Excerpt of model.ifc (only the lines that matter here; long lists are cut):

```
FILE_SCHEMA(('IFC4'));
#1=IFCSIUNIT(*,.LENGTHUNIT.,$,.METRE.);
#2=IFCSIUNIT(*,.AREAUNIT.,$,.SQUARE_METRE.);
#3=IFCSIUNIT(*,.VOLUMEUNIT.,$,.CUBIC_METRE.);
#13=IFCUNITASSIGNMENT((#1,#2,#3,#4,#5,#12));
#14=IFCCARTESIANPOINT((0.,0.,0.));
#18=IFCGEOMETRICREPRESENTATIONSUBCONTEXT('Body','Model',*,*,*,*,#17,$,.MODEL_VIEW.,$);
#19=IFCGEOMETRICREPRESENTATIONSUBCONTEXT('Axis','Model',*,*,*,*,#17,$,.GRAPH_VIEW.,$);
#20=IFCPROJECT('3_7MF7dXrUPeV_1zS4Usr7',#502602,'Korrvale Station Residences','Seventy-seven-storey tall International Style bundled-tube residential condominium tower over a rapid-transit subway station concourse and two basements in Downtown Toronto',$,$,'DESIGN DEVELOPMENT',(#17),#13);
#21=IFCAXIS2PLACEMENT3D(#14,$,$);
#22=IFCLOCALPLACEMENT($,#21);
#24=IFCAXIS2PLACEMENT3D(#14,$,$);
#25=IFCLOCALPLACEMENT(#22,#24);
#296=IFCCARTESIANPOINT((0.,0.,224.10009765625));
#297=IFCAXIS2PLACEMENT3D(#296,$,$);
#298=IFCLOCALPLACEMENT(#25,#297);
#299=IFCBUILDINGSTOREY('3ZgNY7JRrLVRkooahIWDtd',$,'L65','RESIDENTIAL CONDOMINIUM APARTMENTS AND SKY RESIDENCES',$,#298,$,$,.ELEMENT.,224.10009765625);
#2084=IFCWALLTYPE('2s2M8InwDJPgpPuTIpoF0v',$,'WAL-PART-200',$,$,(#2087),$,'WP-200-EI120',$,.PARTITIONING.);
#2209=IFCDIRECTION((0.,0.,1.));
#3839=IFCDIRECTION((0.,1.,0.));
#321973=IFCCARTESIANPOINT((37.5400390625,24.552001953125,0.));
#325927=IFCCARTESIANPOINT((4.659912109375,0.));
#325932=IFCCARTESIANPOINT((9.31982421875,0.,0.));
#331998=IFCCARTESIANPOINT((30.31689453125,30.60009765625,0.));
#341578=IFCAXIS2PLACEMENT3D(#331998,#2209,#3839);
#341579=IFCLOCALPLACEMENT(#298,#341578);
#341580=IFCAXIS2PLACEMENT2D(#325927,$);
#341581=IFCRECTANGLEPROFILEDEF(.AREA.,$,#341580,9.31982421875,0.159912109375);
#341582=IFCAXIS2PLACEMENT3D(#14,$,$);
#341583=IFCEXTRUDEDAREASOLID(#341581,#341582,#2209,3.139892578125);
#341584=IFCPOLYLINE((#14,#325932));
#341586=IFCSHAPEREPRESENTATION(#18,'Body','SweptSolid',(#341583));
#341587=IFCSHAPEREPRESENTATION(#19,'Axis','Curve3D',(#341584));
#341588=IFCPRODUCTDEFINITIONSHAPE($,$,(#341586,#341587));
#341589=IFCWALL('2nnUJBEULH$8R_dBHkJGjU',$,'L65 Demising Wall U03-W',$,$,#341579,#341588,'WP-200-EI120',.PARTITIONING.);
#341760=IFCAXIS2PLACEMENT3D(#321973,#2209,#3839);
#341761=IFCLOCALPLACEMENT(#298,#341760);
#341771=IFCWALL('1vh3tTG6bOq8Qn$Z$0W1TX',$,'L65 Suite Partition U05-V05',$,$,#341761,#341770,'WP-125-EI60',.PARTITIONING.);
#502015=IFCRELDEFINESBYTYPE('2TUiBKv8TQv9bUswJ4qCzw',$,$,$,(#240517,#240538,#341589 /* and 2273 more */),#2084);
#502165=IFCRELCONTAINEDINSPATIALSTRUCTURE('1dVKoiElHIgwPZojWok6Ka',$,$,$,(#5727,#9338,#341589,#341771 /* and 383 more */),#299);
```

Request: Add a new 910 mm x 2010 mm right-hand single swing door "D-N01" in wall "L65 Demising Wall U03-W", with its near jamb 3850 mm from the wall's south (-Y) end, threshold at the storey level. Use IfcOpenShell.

```python
import numpy as np
import ifcopenshell
import ifcopenshell.api.feature
import ifcopenshell.api.geometry
import ifcopenshell.api.root
import ifcopenshell.api.spatial
import ifcopenshell.geom
import ifcopenshell.util.element
import ifcopenshell.util.placement
import ifcopenshell.util.representation
import ifcopenshell.util.shape
import ifcopenshell.util.unit

model = ifcopenshell.open("model.ifc")
unit_scale = ifcopenshell.util.unit.calculate_unit_scale(model)
settings = ifcopenshell.geom.settings()


def volume(element):
    """Net volume in cubic metres, openings subtracted."""
    shape = ifcopenshell.geom.create_shape(settings, element)
    return ifcopenshell.util.shape.get_volume(shape.geometry)


wall = model.by_guid("2nnUJBEULH$8R_dBHkJGjU")
storey = ifcopenshell.util.element.get_container(wall, ifc_class="IfcBuildingStorey")
context = ifcopenshell.util.representation.get_context(model, "Model", "Body", "MODEL_VIEW")
before = volume(wall)

width, height, from_end, sill = 0.91, 2.01, 3.85, 0.0  # metres

# The wall runs along its own X axis, and the end named is its -X end.
wall_shape = ifcopenshell.geom.create_shape(settings, wall)
x, y, z = ifcopenshell.util.shape.get_vertices(wall_shape.geometry).T
start = x.min() + from_end
face, thickness = float(y.min()), float(y.max() - y.min())
wall_matrix = ifcopenshell.util.placement.get_local_placement(wall.ObjectPlacement)
level = ifcopenshell.util.placement.get_local_placement(storey.ObjectPlacement)[2, 3]


def in_wall(x, y):
    """Placement at x, y metres in the wall's axes, at sill height."""
    matrix = wall_matrix.copy()
    matrix[:, 3] = wall_matrix @ np.array([x / unit_scale, y / unit_scale, 0.0, 1.0])
    matrix[2, 3] = level + sill / unit_scale
    return matrix


# Opening: a box that overshoots both wall faces by 50 mm.
opening = ifcopenshell.api.root.create_entity(model, ifc_class="IfcOpeningElement", predefined_type="OPENING")
box = ifcopenshell.api.geometry.add_wall_representation(
    model, context=context, length=width, height=height, thickness=thickness + 0.1
)
ifcopenshell.api.geometry.assign_representation(model, product=opening, representation=box)
ifcopenshell.api.geometry.edit_object_placement(model, product=opening, matrix=in_wall(start, face - 0.05), is_si=False)
ifcopenshell.api.feature.add_feature(model, feature=opening, element=wall)

door = ifcopenshell.api.root.create_entity(model, ifc_class="IfcDoor", name="D-N01", predefined_type="DOOR")
door.OverallWidth, door.OverallHeight = width / unit_scale, height / unit_scale
door.OperationType = "SINGLE_SWING_RIGHT"
body = ifcopenshell.api.geometry.add_door_representation(
    model,
    context=context,
    overall_width=door.OverallWidth,
    overall_height=door.OverallHeight,
    operation_type="SINGLE_SWING_RIGHT",
    lining_properties={"LiningDepth": thickness / unit_scale, "ThresholdDepth": thickness / unit_scale},
)
ifcopenshell.api.geometry.assign_representation(model, product=door, representation=body)
ifcopenshell.api.spatial.assign_container(model, products=[door], relating_structure=storey)
ifcopenshell.api.feature.add_filling(model, opening=opening, element=door)

# The lining spans the wall, so the door starts at the wall face.
ifcopenshell.api.geometry.edit_object_placement(model, product=door, matrix=in_wall(start, face), is_si=False)

after = volume(wall)

print(f"wall volume {before:.3f} -> {after:.3f} m3")

model.write("model_rev.ifc")
```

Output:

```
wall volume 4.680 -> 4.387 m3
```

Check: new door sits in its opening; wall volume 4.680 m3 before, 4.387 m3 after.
